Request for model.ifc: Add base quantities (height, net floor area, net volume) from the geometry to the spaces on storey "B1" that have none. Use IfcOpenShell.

First a look at what the model holds.

```python
import ifcopenshell
import ifcopenshell.util.element
import ifcopenshell.util.unit

model = ifcopenshell.open("model.ifc")
print(model.schema)
for unit_type in ("LENGTHUNIT", "AREAUNIT", "VOLUMEUNIT"):
    print(unit_type, ifcopenshell.util.unit.calculate_unit_scale(model, unit_type))
storey = next(s for s in model.by_type("IfcBuildingStorey") if s.Name == "B1")
spaces = [e for e in ifcopenshell.util.element.get_decomposition(storey) if e.is_a("IfcSpace")]
for e in sorted(spaces, key=lambda e: e.id()):
    print(e.id(), e.is_a(), e.Name, list(ifcopenshell.util.element.get_psets(e, qtos_only=True)), sep=" | ")
```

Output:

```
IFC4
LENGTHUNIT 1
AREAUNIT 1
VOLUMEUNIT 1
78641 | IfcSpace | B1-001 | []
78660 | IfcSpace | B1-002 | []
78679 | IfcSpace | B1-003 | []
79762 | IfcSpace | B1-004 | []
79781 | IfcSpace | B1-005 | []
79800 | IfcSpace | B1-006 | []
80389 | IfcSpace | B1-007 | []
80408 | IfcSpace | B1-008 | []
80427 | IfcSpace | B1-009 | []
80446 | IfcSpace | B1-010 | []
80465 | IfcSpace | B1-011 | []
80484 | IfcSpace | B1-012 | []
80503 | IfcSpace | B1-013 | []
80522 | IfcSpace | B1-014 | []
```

```python
import ifcopenshell
import ifcopenshell.api.pset
import ifcopenshell.geom
import ifcopenshell.util.element
import ifcopenshell.util.shape
import ifcopenshell.util.unit

model = ifcopenshell.open("model.ifc")
unit_scale = ifcopenshell.util.unit.calculate_unit_scale(model)
area_scale = ifcopenshell.util.unit.calculate_unit_scale(model, "AREAUNIT")
volume_scale = ifcopenshell.util.unit.calculate_unit_scale(model, "VOLUMEUNIT")
settings = ifcopenshell.geom.settings()

storey = next(s for s in model.by_type("IfcBuildingStorey") if s.Name == "B1")
spaces = [e for e in ifcopenshell.util.element.get_decomposition(storey) if e.is_a("IfcSpace")]

for e in sorted(spaces, key=lambda e: e.id()):
    if ifcopenshell.util.element.get_psets(e, qtos_only=True, should_inherit=False):
        continue
    # Geometry comes back in metres, in the element's own axes.
    shape = ifcopenshell.geom.create_shape(settings, e)
    values = {
        "Height": ifcopenshell.util.shape.get_z(shape.geometry) / unit_scale,
        "NetFloorArea": ifcopenshell.util.shape.get_footprint_area(shape.geometry) / area_scale,
        "NetVolume": ifcopenshell.util.shape.get_volume(shape.geometry) / volume_scale,
    }
    qto = ifcopenshell.api.pset.add_qto(model, product=e, name="Qto_SpaceBaseQuantities")
    ifcopenshell.api.pset.edit_qto(model, qto=qto, properties=values)
    print(e.id(), {k: round(v, 3) for k, v in values.items()})

model.write("model_edited.ifc")
```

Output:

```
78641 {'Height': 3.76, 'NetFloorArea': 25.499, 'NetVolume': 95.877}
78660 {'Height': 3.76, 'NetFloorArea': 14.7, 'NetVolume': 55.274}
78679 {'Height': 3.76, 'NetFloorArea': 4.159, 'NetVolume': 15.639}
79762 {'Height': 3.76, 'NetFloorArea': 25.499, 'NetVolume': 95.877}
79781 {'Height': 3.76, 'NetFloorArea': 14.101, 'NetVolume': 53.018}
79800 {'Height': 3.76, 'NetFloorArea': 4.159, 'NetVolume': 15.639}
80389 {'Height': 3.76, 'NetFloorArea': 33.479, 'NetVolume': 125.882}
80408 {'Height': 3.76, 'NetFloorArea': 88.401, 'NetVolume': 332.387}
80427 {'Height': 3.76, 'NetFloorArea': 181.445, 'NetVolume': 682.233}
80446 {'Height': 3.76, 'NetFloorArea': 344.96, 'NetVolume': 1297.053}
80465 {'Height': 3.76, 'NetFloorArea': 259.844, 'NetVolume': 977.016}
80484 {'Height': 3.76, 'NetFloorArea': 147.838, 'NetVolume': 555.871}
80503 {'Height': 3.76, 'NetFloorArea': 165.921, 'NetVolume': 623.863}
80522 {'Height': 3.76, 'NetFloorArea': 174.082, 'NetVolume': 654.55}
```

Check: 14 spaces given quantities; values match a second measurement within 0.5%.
